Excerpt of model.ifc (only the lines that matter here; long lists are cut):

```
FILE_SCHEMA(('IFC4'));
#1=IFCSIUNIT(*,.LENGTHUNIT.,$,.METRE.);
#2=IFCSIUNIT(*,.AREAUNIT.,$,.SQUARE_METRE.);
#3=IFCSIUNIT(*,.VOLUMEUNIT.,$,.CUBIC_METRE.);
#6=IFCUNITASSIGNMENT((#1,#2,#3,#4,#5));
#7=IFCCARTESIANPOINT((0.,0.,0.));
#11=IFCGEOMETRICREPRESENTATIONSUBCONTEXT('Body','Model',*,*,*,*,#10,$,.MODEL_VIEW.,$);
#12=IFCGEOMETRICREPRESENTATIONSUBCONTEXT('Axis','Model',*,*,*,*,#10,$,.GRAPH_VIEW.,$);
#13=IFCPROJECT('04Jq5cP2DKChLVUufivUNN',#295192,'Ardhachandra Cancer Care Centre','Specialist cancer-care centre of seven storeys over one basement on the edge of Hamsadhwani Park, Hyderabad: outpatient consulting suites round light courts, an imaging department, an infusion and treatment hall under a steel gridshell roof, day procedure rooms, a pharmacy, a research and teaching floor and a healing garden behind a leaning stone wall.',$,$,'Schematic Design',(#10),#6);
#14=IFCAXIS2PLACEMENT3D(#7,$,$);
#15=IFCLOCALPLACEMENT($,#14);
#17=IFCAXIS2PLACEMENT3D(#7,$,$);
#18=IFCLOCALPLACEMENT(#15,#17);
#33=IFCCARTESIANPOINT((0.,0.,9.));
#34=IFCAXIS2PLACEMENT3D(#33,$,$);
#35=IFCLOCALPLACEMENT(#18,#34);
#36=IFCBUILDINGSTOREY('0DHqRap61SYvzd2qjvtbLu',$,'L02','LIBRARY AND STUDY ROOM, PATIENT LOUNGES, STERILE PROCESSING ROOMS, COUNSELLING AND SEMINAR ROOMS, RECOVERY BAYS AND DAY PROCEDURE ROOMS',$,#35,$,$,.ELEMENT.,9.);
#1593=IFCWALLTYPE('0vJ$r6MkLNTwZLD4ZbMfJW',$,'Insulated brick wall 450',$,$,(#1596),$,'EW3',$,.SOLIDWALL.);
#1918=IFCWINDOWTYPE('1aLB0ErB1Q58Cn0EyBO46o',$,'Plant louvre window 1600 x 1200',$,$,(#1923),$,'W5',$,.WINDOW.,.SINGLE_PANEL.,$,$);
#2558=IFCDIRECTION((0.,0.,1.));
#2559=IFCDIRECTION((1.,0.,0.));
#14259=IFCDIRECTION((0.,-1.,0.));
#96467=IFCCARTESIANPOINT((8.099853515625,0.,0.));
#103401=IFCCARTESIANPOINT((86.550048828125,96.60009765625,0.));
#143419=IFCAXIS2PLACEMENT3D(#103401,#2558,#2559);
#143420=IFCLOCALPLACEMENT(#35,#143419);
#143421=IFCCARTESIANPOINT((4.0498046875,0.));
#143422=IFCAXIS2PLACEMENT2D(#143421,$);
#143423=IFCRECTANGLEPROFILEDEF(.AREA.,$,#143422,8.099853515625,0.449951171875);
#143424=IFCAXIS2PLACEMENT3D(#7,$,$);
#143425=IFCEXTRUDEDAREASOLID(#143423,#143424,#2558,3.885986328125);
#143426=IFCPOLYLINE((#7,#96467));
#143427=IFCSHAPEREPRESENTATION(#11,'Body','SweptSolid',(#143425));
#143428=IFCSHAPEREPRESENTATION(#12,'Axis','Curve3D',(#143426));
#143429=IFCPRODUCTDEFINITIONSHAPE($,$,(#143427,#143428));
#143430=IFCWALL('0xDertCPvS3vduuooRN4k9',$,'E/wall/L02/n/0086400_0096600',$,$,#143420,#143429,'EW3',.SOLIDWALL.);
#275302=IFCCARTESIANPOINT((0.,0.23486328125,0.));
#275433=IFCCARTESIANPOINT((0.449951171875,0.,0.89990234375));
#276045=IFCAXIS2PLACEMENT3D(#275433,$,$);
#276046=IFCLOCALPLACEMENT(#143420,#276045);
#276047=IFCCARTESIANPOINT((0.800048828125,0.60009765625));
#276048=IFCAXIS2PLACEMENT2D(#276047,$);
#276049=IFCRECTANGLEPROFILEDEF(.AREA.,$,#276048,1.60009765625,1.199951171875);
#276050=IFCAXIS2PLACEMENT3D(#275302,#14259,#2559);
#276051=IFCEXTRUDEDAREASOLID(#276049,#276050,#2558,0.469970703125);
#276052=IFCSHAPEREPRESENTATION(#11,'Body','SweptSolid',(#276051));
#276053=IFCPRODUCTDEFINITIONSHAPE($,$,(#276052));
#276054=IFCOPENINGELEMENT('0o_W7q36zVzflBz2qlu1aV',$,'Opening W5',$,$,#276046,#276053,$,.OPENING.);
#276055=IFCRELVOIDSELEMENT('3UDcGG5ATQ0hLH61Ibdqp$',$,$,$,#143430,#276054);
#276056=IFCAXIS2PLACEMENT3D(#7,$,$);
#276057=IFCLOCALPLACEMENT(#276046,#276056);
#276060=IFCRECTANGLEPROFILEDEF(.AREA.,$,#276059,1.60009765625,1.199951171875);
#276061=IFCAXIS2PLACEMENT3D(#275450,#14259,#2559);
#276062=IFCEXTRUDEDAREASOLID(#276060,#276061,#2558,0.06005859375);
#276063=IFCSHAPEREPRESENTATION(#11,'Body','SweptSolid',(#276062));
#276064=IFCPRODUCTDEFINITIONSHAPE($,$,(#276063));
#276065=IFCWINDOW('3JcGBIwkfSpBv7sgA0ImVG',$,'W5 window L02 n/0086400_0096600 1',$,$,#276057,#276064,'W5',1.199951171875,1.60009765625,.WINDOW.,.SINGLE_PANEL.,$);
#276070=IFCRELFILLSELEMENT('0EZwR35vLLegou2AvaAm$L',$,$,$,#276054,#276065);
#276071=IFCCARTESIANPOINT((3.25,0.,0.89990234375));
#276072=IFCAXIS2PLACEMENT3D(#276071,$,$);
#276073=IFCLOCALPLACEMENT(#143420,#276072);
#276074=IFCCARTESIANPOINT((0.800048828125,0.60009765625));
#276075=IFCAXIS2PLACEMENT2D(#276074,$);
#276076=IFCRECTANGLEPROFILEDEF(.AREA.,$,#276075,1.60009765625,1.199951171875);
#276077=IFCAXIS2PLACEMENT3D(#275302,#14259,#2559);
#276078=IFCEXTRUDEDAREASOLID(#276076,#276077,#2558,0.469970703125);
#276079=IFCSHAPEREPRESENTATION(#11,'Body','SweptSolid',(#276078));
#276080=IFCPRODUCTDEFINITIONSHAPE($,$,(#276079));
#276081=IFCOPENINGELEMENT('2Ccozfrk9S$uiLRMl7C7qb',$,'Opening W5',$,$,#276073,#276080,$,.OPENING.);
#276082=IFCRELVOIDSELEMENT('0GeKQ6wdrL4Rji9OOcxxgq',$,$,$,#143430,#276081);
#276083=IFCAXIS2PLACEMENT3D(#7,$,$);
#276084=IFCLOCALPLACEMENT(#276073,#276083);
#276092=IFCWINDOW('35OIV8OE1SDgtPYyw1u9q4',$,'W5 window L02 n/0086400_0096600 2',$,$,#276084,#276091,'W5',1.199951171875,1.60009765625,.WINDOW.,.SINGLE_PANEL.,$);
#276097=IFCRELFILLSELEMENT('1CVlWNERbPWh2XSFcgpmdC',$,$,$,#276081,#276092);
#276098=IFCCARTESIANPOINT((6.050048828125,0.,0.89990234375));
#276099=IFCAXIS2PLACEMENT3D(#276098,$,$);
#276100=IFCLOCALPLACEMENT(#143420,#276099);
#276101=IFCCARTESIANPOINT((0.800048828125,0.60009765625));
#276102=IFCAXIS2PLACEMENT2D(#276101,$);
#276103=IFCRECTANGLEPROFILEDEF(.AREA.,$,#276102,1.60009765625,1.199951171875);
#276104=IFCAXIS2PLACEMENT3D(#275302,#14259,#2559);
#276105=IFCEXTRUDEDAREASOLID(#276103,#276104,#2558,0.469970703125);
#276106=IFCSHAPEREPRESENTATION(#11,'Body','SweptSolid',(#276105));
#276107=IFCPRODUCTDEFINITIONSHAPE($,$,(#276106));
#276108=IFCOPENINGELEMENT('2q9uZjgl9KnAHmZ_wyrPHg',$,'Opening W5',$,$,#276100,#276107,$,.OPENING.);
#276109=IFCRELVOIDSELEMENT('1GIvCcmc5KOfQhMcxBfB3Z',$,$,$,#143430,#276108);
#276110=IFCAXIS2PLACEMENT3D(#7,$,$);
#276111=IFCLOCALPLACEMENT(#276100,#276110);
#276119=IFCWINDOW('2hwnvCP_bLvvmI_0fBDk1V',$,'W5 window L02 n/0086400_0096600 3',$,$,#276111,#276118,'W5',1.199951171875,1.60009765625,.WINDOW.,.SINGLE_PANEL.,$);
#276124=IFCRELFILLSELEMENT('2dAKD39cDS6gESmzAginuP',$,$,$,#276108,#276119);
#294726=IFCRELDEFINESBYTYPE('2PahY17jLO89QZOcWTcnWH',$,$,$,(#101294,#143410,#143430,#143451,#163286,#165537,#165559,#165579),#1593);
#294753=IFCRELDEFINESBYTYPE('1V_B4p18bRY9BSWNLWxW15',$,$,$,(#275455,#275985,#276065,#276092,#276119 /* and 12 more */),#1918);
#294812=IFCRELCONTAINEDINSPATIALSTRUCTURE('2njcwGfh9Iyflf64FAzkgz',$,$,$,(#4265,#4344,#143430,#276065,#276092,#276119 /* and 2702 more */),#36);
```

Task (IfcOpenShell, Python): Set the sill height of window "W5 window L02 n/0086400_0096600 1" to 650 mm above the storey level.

```python
import numpy as np
import ifcopenshell
import ifcopenshell.api.geometry
import ifcopenshell.geom
import ifcopenshell.util.element
import ifcopenshell.util.placement
import ifcopenshell.util.shape
import ifcopenshell.util.unit

model = ifcopenshell.open("model.ifc")
unit_scale = ifcopenshell.util.unit.calculate_unit_scale(model)

window = model.by_id(276065)
opening = window.FillsVoids[0].RelatingOpeningElement
storey = ifcopenshell.util.element.get_container(window, ifc_class="IfcBuildingStorey")
level = ifcopenshell.util.placement.get_local_placement(storey.ObjectPlacement)[2, 3]

# The opening's origin need not be at the sill, so measure its lowest point.
shape = ifcopenshell.geom.create_shape(ifcopenshell.geom.settings(), opening)
bottom = ifcopenshell.util.shape.get_shape_bottom_elevation(shape, shape.geometry) / unit_scale
dz = level + 0.65 - bottom

shift = np.array([0.0, 0.0, dz])
# The window is placed relative to its opening, so it follows when the opening moves.
matrix = ifcopenshell.util.placement.get_local_placement(opening.ObjectPlacement)
matrix[:3, 3] += shift
ifcopenshell.api.geometry.edit_object_placement(
    model, product=opening, matrix=matrix, is_si=False, should_transform_children=True
)

print(f"moved by {dz * unit_scale:+.3f} m")

model.write("model-out.ifc")
```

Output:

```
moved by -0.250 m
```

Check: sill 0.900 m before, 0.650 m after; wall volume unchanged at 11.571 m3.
